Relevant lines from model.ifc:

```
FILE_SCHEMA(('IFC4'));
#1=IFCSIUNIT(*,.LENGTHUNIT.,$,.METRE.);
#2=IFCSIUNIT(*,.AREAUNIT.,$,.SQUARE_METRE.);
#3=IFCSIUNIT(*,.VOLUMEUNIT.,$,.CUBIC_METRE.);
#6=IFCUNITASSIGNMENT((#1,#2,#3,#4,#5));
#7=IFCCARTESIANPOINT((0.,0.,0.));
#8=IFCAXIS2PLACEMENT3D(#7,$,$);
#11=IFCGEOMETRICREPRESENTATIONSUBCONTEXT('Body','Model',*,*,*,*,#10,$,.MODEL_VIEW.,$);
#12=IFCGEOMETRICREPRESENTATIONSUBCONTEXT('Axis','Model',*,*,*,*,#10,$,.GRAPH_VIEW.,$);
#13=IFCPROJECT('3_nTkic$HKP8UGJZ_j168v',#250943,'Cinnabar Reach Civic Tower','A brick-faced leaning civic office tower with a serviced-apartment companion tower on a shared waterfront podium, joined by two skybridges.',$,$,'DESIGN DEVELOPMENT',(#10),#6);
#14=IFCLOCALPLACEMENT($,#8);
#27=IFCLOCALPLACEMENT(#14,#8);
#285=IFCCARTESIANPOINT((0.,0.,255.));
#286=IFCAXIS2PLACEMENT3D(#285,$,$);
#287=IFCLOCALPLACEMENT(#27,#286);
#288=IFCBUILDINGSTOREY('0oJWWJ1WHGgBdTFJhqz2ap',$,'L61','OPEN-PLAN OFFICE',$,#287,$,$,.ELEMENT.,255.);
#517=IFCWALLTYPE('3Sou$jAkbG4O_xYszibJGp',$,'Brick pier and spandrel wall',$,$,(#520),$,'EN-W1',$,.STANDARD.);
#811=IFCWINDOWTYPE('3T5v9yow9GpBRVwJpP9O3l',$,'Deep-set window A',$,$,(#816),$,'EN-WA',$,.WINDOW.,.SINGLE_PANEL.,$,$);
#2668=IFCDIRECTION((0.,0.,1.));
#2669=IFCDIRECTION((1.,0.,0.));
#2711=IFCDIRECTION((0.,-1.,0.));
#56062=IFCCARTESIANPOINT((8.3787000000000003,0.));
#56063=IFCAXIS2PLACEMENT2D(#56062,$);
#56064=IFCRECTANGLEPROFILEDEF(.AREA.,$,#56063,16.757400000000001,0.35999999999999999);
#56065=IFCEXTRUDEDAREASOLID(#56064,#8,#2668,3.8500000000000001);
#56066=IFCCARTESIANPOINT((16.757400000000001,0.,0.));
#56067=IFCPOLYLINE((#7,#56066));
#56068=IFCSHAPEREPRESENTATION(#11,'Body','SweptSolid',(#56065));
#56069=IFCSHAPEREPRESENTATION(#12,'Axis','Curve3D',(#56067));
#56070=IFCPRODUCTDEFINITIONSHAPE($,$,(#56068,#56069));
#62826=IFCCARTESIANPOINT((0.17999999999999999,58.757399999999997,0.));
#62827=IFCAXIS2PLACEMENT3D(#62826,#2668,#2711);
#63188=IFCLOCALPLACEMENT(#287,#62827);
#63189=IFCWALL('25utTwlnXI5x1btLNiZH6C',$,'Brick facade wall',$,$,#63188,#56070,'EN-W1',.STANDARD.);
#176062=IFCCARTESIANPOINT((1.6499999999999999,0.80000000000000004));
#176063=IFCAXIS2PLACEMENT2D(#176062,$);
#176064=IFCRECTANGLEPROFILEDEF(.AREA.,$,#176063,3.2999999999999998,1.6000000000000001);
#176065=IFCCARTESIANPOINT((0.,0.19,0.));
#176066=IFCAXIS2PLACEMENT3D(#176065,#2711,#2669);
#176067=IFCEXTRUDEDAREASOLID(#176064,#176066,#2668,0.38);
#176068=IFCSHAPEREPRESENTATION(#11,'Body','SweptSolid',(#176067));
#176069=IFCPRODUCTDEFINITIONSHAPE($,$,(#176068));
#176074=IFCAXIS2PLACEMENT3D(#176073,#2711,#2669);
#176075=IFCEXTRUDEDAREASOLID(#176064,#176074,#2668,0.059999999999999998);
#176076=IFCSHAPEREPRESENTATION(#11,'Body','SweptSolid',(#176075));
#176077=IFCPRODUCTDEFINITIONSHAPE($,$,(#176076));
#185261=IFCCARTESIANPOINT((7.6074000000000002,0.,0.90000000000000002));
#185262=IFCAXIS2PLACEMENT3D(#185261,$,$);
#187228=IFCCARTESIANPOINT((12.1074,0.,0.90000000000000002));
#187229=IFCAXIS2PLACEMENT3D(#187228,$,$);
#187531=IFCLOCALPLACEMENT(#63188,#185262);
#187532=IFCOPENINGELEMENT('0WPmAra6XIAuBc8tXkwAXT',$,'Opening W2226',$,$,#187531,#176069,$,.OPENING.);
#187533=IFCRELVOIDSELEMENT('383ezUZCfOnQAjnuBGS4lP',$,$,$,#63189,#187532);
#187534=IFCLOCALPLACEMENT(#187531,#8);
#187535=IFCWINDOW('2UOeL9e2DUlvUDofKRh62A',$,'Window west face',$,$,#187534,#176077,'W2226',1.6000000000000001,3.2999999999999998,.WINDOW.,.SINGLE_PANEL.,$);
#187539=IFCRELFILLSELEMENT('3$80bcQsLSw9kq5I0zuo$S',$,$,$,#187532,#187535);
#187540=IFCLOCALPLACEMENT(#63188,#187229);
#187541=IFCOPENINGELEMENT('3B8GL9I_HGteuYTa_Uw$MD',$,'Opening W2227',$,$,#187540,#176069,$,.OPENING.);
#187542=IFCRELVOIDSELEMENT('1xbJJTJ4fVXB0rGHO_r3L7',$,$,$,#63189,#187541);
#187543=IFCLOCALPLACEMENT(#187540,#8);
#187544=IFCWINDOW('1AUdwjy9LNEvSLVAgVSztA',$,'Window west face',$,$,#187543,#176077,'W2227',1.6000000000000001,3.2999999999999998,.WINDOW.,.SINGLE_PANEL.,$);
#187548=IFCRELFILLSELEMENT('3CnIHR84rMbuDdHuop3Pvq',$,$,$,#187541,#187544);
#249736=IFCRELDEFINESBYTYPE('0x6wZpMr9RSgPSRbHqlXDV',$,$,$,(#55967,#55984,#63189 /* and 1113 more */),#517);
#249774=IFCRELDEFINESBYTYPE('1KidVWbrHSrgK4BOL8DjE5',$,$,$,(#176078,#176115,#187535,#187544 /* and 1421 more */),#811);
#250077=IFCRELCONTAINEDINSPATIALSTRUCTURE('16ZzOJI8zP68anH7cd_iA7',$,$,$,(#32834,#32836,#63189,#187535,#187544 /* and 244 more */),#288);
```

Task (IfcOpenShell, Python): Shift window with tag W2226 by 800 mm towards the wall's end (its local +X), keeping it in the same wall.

```python
import ifcopenshell
import ifcopenshell.api.geometry
import ifcopenshell.util.placement
import ifcopenshell.util.unit

model = ifcopenshell.open("model.ifc")
unit_scale = ifcopenshell.util.unit.calculate_unit_scale(model)

window = model.by_guid("2UOeL9e2DUlvUDofKRh62A")
opening = window.FillsVoids[0].RelatingOpeningElement
wall = opening.VoidsElements[0].RelatingBuildingElement

wall_matrix = ifcopenshell.util.placement.get_local_placement(wall.ObjectPlacement)
shift = wall_matrix[:3, 0] * 0.8 / unit_scale
before = ifcopenshell.util.placement.get_local_placement(window.ObjectPlacement)[:3, 3].copy()

# The window is placed relative to its opening, so it follows when the opening moves.
matrix = ifcopenshell.util.placement.get_local_placement(opening.ObjectPlacement)
matrix[:3, 3] += shift
ifcopenshell.api.geometry.edit_object_placement(
    model, product=opening, matrix=matrix, is_si=False, should_transform_children=True
)

after = ifcopenshell.util.placement.get_local_placement(window.ObjectPlacement)[:3, 3]
print("window moved by", (after - before).round(3) + 0.0)

model.write("model_v2.ifc")
```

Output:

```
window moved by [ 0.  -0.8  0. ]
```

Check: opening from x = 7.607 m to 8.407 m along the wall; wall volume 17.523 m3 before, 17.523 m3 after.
